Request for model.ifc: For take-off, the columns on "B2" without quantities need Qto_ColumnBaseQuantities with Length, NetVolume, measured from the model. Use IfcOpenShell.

First a look at what the model holds.

```python
import ifcopenshell
import ifcopenshell.util.element
import ifcopenshell.util.unit

model = ifcopenshell.open("model.ifc")
print(model.schema)
for unit_type in ("LENGTHUNIT", "AREAUNIT", "VOLUMEUNIT"):
    print(unit_type, ifcopenshell.util.unit.calculate_unit_scale(model, unit_type))
storey = next(s for s in model.by_type("IfcBuildingStorey") if s.Name == "B2")
columns = [e for e in ifcopenshell.util.element.get_decomposition(storey) if e.is_a("IfcColumn")]
for e in sorted(columns, key=lambda e: e.id()):
    print(e.id(), e.is_a(), e.Name, list(ifcopenshell.util.element.get_psets(e, qtos_only=True)), sep=" | ")
```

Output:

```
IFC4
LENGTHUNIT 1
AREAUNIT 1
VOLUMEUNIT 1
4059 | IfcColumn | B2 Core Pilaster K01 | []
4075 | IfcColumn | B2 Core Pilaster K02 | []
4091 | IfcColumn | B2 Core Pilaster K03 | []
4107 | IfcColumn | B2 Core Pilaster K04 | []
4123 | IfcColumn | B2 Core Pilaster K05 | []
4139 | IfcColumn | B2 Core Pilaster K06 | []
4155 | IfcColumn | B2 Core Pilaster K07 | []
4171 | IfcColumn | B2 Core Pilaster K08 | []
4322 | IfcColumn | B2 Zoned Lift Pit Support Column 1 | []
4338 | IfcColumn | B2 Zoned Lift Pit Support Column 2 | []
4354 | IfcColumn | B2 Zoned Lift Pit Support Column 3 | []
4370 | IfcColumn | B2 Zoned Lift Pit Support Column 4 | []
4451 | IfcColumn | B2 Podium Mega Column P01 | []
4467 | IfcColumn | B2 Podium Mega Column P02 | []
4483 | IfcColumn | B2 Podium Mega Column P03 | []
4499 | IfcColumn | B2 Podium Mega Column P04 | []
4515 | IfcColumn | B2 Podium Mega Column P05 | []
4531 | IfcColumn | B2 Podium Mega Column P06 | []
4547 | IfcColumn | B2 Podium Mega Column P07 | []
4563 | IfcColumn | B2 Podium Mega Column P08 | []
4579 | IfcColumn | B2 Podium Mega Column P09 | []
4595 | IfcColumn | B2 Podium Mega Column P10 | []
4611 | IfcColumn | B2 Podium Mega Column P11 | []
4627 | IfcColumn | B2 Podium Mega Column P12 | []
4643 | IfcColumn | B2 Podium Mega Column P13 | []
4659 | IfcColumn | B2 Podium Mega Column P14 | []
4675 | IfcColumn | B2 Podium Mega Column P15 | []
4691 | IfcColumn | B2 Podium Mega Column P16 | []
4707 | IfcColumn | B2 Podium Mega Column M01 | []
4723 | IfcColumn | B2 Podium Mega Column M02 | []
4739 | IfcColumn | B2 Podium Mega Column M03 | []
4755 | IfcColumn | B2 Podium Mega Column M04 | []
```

```python
import ifcopenshell
import ifcopenshell.api.pset
import ifcopenshell.geom
import ifcopenshell.util.element
import ifcopenshell.util.shape
import ifcopenshell.util.unit

model = ifcopenshell.open("model.ifc")
unit_scale = ifcopenshell.util.unit.calculate_unit_scale(model)
volume_scale = ifcopenshell.util.unit.calculate_unit_scale(model, "VOLUMEUNIT")
settings = ifcopenshell.geom.settings()

storey = next(s for s in model.by_type("IfcBuildingStorey") if s.Name == "B2")
columns = [e for e in ifcopenshell.util.element.get_decomposition(storey) if e.is_a("IfcColumn")]

for e in sorted(columns, key=lambda e: e.id()):
    if ifcopenshell.util.element.get_psets(e, qtos_only=True, should_inherit=False):
        continue
    # Geometry comes back in metres, in the element's own axes.
    shape = ifcopenshell.geom.create_shape(settings, e)
    values = {
        "Length": ifcopenshell.util.shape.get_z(shape.geometry) / unit_scale,
        "NetVolume": ifcopenshell.util.shape.get_volume(shape.geometry) / volume_scale,
    }
    qto = ifcopenshell.api.pset.add_qto(model, product=e, name="Qto_ColumnBaseQuantities")
    ifcopenshell.api.pset.edit_qto(model, qto=qto, properties=values)
    print(e.id(), {k: round(v, 3) for k, v in values.items()})

model.write("model_rev.ifc")
```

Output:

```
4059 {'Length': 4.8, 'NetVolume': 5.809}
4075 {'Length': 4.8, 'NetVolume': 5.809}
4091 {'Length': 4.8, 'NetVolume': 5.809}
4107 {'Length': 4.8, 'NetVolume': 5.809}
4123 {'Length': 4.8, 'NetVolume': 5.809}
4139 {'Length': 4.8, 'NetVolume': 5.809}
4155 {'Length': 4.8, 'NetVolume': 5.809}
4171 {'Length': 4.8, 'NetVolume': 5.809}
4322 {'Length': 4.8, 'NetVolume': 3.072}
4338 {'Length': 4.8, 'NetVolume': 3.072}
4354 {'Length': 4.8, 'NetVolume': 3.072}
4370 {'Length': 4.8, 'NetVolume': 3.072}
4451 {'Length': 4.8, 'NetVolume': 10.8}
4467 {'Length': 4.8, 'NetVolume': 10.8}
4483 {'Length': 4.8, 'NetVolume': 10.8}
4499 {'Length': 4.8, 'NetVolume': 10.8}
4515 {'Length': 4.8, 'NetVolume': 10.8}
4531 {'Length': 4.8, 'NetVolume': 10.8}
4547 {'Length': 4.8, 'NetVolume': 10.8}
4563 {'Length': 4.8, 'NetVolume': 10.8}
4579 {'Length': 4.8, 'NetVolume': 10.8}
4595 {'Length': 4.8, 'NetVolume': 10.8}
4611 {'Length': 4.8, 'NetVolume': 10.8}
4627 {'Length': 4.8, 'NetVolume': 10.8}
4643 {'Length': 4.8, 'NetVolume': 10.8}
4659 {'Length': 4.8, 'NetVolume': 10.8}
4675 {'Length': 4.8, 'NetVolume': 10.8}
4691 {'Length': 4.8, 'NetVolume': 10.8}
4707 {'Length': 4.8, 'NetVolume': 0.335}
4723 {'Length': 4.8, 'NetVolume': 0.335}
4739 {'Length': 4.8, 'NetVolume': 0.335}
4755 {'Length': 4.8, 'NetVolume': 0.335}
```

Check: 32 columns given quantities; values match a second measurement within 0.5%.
